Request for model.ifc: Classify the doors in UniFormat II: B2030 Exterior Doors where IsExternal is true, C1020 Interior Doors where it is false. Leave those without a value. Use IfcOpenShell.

First a look at what the model holds.

```python
import ifcopenshell
import ifcopenshell.util.element

model = ifcopenshell.open("model.ifc")
print(model.schema)
print("classifications:", [c.Name for c in model.by_type("IfcClassification")])
values = [ifcopenshell.util.element.get_pset(e, "Pset_DoorCommon", "IsExternal") for e in model.by_type("IfcDoor")]
for value in (True, False, None):
    print("IsExternal", value, values.count(value))
```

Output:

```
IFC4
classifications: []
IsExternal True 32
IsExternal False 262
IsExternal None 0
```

```python
import ifcopenshell
import ifcopenshell.api.classification
import ifcopenshell.util.element

model = ifcopenshell.open("model.ifc")

system = ifcopenshell.api.classification.add_classification(model, classification="UniFormat II")

doors = model.by_type("IfcDoor")
external = {e: ifcopenshell.util.element.get_pset(e, "Pset_DoorCommon", "IsExternal") for e in doors}
for flag, code, name in ((True, "B2030", "Exterior Doors"), (False, "C1020", "Interior Doors")):
    products = [e for e in doors if external[e] is flag]
    ifcopenshell.api.classification.add_reference(
        model, products=products, classification=system, identification=code, name=name
    )
    print(code, len(products))

model.write("model_edited.ifc")
```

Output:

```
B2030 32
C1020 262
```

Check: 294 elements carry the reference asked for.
